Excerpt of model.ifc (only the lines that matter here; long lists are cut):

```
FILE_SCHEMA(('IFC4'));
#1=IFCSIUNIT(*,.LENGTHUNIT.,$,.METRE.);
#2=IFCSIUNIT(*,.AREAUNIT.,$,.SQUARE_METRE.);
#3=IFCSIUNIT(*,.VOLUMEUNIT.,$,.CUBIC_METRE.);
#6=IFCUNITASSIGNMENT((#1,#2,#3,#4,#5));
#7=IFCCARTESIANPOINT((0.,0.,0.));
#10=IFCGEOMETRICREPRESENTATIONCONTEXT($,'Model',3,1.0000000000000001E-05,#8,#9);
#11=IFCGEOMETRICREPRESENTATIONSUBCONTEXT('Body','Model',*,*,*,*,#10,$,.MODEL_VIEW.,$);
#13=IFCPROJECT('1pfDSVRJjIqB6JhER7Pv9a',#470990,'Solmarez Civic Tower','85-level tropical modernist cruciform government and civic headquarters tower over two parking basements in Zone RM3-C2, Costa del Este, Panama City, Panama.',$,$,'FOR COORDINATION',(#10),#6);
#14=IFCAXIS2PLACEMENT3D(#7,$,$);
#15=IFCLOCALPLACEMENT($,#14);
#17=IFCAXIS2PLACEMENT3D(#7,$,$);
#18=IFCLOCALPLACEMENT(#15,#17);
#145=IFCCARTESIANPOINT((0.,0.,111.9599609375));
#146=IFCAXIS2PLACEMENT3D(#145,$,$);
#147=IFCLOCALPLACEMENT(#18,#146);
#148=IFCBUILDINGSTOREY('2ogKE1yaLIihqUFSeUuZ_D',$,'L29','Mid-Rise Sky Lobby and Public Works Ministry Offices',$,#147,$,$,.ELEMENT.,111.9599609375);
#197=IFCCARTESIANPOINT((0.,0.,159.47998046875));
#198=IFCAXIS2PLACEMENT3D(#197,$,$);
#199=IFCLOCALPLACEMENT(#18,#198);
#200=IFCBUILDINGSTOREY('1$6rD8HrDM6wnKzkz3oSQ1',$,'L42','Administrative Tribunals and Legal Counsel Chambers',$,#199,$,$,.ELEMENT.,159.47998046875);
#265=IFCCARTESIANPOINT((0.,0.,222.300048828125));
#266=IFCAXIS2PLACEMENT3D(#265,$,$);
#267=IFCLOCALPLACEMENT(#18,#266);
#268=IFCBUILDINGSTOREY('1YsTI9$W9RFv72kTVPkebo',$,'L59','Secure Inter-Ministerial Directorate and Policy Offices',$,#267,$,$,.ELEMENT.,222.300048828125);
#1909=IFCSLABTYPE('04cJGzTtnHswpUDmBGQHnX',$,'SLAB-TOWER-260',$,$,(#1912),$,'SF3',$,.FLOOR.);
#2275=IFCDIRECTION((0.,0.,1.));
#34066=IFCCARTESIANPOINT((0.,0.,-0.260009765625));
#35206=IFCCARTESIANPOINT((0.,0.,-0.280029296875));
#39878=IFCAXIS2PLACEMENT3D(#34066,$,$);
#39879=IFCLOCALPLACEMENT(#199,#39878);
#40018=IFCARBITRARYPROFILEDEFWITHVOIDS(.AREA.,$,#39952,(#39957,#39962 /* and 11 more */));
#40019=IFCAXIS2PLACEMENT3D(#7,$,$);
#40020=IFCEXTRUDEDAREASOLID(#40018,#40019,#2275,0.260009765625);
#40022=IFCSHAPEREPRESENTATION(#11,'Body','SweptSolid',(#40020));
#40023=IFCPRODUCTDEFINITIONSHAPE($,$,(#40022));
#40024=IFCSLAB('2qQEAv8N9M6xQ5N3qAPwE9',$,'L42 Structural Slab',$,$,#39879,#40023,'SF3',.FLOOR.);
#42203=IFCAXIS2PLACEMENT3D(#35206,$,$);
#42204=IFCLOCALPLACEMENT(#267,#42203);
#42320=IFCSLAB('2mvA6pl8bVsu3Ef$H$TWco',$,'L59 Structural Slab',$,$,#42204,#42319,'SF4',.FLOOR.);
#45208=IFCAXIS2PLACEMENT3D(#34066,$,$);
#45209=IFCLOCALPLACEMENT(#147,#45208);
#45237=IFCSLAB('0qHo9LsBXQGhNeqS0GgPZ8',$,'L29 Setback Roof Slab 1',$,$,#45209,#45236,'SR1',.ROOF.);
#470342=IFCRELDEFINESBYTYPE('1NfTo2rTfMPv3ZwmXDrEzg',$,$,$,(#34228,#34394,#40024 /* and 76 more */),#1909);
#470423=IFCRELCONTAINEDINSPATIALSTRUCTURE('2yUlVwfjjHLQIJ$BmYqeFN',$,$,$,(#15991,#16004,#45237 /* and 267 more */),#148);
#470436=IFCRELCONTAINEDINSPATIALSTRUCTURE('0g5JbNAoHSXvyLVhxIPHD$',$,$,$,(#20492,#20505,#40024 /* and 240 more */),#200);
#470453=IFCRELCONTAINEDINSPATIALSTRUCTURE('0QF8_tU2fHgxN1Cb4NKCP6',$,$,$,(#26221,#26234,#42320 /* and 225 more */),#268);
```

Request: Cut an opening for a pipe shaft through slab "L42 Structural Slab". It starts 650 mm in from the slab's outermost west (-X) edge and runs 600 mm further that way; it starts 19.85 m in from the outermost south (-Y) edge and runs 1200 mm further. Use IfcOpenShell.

```python
import numpy as np
import ifcopenshell
import ifcopenshell.api.feature
import ifcopenshell.api.geometry
import ifcopenshell.api.root
import ifcopenshell.geom
import ifcopenshell.util.placement
import ifcopenshell.util.representation
import ifcopenshell.util.shape
import ifcopenshell.util.unit

model = ifcopenshell.open("model.ifc")
unit_scale = ifcopenshell.util.unit.calculate_unit_scale(model)
settings = ifcopenshell.geom.settings()


def volume(element):
    """Net volume in cubic metres, openings subtracted."""
    shape = ifcopenshell.geom.create_shape(settings, element)
    return ifcopenshell.util.shape.get_volume(shape.geometry)


slab = model.by_guid("2qQEAv8N9M6xQ5N3qAPwE9")
before = volume(slab)

# Extent in the slab's own axes, in metres. The edges named are its -X and -Y sides.
slab_shape = ifcopenshell.geom.create_shape(settings, slab)
vertices = ifcopenshell.util.shape.get_vertices(slab_shape.geometry)
x_min, y_min, bottom = vertices.min(axis=0)
top = vertices[:, 2].max()

opening = ifcopenshell.api.root.create_entity(model, ifc_class="IfcOpeningElement", name="Pipe shaft opening", predefined_type="OPENING")
context = ifcopenshell.util.representation.get_context(model, "Model", "Body", "MODEL_VIEW")
width, depth = 0.6, 1.2
outline = [(0.0, 0.0), (width, 0.0), (width, depth), (0.0, depth), (0.0, 0.0)]
# Overshoot both faces by 50 mm so the cut is clean.
shape = ifcopenshell.api.geometry.add_slab_representation(
    model, context=context, depth=top - bottom + 0.1, polyline=outline
)
ifcopenshell.api.geometry.assign_representation(model, product=opening, representation=shape)

matrix = ifcopenshell.util.placement.get_local_placement(slab.ObjectPlacement)
matrix[:, 3] = matrix @ np.append(np.array([x_min + 0.65, y_min + 19.85, bottom - 0.05]) / unit_scale, 1.0)
ifcopenshell.api.geometry.edit_object_placement(model, product=opening, matrix=matrix, is_si=False)
ifcopenshell.api.feature.add_feature(model, feature=opening, element=slab)

after = volume(slab)

print(f"slab volume {before:.3f} -> {after:.3f} m3")

model.write("model_edited.ifc")
```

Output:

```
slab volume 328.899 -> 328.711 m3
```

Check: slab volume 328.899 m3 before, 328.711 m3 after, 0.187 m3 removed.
